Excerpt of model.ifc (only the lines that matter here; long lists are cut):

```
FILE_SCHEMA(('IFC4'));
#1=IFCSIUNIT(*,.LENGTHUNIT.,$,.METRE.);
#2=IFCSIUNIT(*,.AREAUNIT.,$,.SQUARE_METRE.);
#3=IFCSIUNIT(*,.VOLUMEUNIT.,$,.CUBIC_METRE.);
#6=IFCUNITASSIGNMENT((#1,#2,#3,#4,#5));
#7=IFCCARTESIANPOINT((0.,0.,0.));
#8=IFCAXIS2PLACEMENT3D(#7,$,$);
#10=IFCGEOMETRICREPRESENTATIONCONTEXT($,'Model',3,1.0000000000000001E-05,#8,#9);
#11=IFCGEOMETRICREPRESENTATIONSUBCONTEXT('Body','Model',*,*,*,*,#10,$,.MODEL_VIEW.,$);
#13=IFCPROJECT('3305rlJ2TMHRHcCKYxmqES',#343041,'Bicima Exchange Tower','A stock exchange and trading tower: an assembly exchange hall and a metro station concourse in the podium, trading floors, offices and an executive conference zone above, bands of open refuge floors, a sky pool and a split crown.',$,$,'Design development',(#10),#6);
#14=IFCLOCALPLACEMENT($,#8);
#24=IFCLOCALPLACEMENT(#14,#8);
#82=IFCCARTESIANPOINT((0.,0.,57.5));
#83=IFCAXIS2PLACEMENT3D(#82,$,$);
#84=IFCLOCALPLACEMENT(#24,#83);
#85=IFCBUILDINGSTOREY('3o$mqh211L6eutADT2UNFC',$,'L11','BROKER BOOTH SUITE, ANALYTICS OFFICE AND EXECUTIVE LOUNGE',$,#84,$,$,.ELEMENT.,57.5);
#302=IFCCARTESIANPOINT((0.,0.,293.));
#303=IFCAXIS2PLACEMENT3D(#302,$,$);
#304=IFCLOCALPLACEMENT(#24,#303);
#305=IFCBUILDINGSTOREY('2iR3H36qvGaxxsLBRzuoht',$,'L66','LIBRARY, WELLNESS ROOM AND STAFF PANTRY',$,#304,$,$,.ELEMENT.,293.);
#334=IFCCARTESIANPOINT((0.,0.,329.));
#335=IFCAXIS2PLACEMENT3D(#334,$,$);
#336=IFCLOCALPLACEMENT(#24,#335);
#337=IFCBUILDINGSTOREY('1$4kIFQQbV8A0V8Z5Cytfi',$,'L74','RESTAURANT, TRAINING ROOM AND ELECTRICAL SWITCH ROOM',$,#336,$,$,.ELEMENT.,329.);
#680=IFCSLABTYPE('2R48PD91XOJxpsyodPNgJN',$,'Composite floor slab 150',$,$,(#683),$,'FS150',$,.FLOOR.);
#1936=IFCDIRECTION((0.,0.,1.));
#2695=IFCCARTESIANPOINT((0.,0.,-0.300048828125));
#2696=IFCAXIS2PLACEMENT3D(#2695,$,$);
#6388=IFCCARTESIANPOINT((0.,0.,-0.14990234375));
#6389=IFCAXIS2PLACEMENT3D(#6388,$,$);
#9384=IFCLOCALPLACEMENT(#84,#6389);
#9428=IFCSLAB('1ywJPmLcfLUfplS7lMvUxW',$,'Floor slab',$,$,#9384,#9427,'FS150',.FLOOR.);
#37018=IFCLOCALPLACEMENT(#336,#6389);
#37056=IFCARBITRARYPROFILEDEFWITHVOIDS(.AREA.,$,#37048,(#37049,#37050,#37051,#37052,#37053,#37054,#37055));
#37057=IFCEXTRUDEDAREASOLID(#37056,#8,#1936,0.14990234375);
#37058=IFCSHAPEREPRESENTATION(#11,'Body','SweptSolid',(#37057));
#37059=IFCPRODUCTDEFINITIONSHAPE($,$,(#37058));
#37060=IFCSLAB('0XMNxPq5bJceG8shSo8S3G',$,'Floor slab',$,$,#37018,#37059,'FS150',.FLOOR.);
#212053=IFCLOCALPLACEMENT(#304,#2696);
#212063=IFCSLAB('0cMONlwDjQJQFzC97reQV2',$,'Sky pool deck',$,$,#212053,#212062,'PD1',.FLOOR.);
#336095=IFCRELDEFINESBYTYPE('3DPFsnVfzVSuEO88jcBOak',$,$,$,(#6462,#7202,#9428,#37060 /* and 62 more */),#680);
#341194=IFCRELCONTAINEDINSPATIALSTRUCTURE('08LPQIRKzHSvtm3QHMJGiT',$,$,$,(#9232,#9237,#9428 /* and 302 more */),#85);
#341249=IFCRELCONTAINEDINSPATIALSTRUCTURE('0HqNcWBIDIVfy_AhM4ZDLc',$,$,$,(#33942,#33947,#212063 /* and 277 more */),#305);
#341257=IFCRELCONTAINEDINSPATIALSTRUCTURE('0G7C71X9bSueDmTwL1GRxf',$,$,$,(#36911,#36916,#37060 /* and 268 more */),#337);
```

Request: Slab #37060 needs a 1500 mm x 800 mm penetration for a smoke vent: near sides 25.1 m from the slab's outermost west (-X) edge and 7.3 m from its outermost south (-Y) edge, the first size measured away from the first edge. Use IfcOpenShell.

```python
import numpy as np
import ifcopenshell
import ifcopenshell.api.feature
import ifcopenshell.api.geometry
import ifcopenshell.api.root
import ifcopenshell.geom
import ifcopenshell.util.placement
import ifcopenshell.util.representation
import ifcopenshell.util.shape
import ifcopenshell.util.unit

model = ifcopenshell.open("model.ifc")
unit_scale = ifcopenshell.util.unit.calculate_unit_scale(model)
settings = ifcopenshell.geom.settings()


def volume(element):
    """Net volume in cubic metres, openings subtracted."""
    shape = ifcopenshell.geom.create_shape(settings, element)
    return ifcopenshell.util.shape.get_volume(shape.geometry)


slab = model.by_guid("0XMNxPq5bJceG8shSo8S3G")
before = volume(slab)

# Extent in the slab's own axes, in metres. The edges named are its -X and -Y sides.
slab_shape = ifcopenshell.geom.create_shape(settings, slab)
vertices = ifcopenshell.util.shape.get_vertices(slab_shape.geometry)
x_min, y_min, bottom = vertices.min(axis=0)
top = vertices[:, 2].max()

opening = ifcopenshell.api.root.create_entity(model, ifc_class="IfcOpeningElement", name="Smoke vent opening", predefined_type="OPENING")
context = ifcopenshell.util.representation.get_context(model, "Model", "Body", "MODEL_VIEW")
width, depth = 1.5, 0.8
outline = [(0.0, 0.0), (width, 0.0), (width, depth), (0.0, depth), (0.0, 0.0)]
# Overshoot both faces by 50 mm so the cut is clean.
shape = ifcopenshell.api.geometry.add_slab_representation(
    model, context=context, depth=top - bottom + 0.1, polyline=outline
)
ifcopenshell.api.geometry.assign_representation(model, product=opening, representation=shape)

matrix = ifcopenshell.util.placement.get_local_placement(slab.ObjectPlacement)
matrix[:, 3] = matrix @ np.append(np.array([x_min + 25.1, y_min + 7.3, bottom - 0.05]) / unit_scale, 1.0)
ifcopenshell.api.geometry.edit_object_placement(model, product=opening, matrix=matrix, is_si=False)
ifcopenshell.api.feature.add_feature(model, feature=opening, element=slab)

after = volume(slab)

print(f"slab volume {before:.3f} -> {after:.3f} m3")

model.write("model-out.ifc")
```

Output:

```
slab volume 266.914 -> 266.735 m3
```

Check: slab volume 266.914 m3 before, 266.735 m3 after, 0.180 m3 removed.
